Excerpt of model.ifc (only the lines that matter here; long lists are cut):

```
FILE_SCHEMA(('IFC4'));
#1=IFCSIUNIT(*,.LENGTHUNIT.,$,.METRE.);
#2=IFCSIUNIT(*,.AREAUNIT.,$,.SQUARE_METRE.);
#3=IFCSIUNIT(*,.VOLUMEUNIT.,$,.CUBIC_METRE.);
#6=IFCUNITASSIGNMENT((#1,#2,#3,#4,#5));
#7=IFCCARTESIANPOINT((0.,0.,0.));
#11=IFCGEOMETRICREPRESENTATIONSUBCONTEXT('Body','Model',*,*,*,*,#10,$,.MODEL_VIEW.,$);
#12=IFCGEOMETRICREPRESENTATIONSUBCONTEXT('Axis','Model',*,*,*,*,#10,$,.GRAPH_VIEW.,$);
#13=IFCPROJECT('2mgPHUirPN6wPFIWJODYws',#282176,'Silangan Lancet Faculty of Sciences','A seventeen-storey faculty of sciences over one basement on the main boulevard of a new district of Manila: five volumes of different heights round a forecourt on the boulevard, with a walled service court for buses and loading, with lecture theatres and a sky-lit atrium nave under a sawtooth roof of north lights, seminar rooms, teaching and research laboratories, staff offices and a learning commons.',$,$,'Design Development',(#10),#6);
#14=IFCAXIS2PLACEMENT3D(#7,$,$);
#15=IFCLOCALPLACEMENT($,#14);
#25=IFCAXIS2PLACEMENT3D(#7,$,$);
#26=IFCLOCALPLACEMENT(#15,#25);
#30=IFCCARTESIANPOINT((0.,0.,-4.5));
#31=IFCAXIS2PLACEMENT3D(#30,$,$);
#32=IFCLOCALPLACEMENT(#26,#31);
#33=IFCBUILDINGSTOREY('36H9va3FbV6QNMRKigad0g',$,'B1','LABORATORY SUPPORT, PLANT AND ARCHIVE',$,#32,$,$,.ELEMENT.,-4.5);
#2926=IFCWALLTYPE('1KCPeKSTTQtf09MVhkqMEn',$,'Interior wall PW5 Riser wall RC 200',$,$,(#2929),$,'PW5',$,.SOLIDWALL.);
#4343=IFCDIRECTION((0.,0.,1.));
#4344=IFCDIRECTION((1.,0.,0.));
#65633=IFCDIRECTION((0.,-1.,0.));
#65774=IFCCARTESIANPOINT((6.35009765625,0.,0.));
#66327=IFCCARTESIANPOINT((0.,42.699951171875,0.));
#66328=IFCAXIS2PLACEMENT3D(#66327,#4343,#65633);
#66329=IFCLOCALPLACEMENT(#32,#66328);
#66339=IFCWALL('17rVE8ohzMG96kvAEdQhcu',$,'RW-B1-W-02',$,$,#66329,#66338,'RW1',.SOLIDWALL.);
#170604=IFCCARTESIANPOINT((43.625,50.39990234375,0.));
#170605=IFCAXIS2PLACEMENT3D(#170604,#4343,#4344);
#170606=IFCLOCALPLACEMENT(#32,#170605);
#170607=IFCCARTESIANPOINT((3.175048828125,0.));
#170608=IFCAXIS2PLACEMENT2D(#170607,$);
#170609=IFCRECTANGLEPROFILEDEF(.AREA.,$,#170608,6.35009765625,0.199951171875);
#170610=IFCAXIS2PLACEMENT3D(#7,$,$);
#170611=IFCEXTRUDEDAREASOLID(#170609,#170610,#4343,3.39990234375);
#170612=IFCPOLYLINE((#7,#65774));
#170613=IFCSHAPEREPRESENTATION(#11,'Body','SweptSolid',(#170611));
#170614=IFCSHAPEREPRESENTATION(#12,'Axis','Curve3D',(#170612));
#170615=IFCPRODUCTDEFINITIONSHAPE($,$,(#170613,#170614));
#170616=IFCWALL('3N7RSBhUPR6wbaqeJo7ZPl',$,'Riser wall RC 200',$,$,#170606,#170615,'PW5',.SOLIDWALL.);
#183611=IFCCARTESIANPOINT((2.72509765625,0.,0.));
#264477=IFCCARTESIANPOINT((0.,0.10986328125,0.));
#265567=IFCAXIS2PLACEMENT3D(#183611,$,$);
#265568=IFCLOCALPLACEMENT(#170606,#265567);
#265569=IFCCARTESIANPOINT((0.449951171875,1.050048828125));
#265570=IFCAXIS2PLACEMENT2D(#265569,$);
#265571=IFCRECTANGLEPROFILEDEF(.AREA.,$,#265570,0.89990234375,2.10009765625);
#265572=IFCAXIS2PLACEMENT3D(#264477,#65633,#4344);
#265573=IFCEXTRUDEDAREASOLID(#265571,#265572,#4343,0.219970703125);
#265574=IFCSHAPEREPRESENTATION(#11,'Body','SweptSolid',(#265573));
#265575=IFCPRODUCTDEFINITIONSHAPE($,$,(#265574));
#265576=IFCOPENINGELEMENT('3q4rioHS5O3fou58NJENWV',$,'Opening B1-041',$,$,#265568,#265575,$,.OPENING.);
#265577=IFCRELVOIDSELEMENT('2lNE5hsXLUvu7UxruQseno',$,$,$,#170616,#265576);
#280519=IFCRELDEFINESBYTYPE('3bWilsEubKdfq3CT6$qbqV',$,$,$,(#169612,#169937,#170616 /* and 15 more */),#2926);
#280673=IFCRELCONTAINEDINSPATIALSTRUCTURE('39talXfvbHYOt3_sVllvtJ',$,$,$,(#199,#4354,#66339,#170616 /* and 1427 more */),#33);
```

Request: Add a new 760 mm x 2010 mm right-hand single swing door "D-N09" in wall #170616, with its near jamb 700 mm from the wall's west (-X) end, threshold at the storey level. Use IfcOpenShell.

```python
import numpy as np
import ifcopenshell
import ifcopenshell.api.feature
import ifcopenshell.api.geometry
import ifcopenshell.api.root
import ifcopenshell.api.spatial
import ifcopenshell.geom
import ifcopenshell.util.element
import ifcopenshell.util.placement
import ifcopenshell.util.representation
import ifcopenshell.util.shape
import ifcopenshell.util.unit

model = ifcopenshell.open("model.ifc")
unit_scale = ifcopenshell.util.unit.calculate_unit_scale(model)
settings = ifcopenshell.geom.settings()


def volume(element):
    """Net volume in cubic metres, openings subtracted."""
    shape = ifcopenshell.geom.create_shape(settings, element)
    return ifcopenshell.util.shape.get_volume(shape.geometry)


wall = model.by_id(170616)
storey = ifcopenshell.util.element.get_container(wall, ifc_class="IfcBuildingStorey")
context = ifcopenshell.util.representation.get_context(model, "Model", "Body", "MODEL_VIEW")
before = volume(wall)

width, height, from_end, sill = 0.76, 2.01, 0.7, 0.0  # metres

# The wall runs along its own X axis, and the end named is its -X end.
wall_shape = ifcopenshell.geom.create_shape(settings, wall)
x, y, z = ifcopenshell.util.shape.get_vertices(wall_shape.geometry).T
start = x.min() + from_end
face, thickness = float(y.min()), float(y.max() - y.min())
wall_matrix = ifcopenshell.util.placement.get_local_placement(wall.ObjectPlacement)
level = ifcopenshell.util.placement.get_local_placement(storey.ObjectPlacement)[2, 3]


def in_wall(x, y):
    """Placement at x, y metres in the wall's axes, at sill height."""
    matrix = wall_matrix.copy()
    matrix[:, 3] = wall_matrix @ np.array([x / unit_scale, y / unit_scale, 0.0, 1.0])
    matrix[2, 3] = level + sill / unit_scale
    return matrix


# Opening: a box that overshoots both wall faces by 50 mm.
opening = ifcopenshell.api.root.create_entity(model, ifc_class="IfcOpeningElement", predefined_type="OPENING")
box = ifcopenshell.api.geometry.add_wall_representation(
    model, context=context, length=width, height=height, thickness=thickness + 0.1
)
ifcopenshell.api.geometry.assign_representation(model, product=opening, representation=box)
ifcopenshell.api.geometry.edit_object_placement(model, product=opening, matrix=in_wall(start, face - 0.05), is_si=False)
ifcopenshell.api.feature.add_feature(model, feature=opening, element=wall)

door = ifcopenshell.api.root.create_entity(model, ifc_class="IfcDoor", name="D-N09", predefined_type="DOOR")
door.OverallWidth, door.OverallHeight = width / unit_scale, height / unit_scale
door.OperationType = "SINGLE_SWING_RIGHT"
body = ifcopenshell.api.geometry.add_door_representation(
    model,
    context=context,
    overall_width=door.OverallWidth,
    overall_height=door.OverallHeight,
    operation_type="SINGLE_SWING_RIGHT",
    lining_properties={"LiningDepth": thickness / unit_scale, "ThresholdDepth": thickness / unit_scale},
)
ifcopenshell.api.geometry.assign_representation(model, product=door, representation=body)
ifcopenshell.api.spatial.assign_container(model, products=[door], relating_structure=storey)
ifcopenshell.api.feature.add_filling(model, opening=opening, element=door)

# The lining spans the wall, so the door starts at the wall face.
ifcopenshell.api.geometry.edit_object_placement(model, product=door, matrix=in_wall(start, face), is_si=False)

after = volume(wall)

print(f"wall volume {before:.3f} -> {after:.3f} m3")

model.write("model_edited.ifc")
```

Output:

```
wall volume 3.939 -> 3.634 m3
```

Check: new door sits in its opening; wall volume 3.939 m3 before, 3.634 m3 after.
